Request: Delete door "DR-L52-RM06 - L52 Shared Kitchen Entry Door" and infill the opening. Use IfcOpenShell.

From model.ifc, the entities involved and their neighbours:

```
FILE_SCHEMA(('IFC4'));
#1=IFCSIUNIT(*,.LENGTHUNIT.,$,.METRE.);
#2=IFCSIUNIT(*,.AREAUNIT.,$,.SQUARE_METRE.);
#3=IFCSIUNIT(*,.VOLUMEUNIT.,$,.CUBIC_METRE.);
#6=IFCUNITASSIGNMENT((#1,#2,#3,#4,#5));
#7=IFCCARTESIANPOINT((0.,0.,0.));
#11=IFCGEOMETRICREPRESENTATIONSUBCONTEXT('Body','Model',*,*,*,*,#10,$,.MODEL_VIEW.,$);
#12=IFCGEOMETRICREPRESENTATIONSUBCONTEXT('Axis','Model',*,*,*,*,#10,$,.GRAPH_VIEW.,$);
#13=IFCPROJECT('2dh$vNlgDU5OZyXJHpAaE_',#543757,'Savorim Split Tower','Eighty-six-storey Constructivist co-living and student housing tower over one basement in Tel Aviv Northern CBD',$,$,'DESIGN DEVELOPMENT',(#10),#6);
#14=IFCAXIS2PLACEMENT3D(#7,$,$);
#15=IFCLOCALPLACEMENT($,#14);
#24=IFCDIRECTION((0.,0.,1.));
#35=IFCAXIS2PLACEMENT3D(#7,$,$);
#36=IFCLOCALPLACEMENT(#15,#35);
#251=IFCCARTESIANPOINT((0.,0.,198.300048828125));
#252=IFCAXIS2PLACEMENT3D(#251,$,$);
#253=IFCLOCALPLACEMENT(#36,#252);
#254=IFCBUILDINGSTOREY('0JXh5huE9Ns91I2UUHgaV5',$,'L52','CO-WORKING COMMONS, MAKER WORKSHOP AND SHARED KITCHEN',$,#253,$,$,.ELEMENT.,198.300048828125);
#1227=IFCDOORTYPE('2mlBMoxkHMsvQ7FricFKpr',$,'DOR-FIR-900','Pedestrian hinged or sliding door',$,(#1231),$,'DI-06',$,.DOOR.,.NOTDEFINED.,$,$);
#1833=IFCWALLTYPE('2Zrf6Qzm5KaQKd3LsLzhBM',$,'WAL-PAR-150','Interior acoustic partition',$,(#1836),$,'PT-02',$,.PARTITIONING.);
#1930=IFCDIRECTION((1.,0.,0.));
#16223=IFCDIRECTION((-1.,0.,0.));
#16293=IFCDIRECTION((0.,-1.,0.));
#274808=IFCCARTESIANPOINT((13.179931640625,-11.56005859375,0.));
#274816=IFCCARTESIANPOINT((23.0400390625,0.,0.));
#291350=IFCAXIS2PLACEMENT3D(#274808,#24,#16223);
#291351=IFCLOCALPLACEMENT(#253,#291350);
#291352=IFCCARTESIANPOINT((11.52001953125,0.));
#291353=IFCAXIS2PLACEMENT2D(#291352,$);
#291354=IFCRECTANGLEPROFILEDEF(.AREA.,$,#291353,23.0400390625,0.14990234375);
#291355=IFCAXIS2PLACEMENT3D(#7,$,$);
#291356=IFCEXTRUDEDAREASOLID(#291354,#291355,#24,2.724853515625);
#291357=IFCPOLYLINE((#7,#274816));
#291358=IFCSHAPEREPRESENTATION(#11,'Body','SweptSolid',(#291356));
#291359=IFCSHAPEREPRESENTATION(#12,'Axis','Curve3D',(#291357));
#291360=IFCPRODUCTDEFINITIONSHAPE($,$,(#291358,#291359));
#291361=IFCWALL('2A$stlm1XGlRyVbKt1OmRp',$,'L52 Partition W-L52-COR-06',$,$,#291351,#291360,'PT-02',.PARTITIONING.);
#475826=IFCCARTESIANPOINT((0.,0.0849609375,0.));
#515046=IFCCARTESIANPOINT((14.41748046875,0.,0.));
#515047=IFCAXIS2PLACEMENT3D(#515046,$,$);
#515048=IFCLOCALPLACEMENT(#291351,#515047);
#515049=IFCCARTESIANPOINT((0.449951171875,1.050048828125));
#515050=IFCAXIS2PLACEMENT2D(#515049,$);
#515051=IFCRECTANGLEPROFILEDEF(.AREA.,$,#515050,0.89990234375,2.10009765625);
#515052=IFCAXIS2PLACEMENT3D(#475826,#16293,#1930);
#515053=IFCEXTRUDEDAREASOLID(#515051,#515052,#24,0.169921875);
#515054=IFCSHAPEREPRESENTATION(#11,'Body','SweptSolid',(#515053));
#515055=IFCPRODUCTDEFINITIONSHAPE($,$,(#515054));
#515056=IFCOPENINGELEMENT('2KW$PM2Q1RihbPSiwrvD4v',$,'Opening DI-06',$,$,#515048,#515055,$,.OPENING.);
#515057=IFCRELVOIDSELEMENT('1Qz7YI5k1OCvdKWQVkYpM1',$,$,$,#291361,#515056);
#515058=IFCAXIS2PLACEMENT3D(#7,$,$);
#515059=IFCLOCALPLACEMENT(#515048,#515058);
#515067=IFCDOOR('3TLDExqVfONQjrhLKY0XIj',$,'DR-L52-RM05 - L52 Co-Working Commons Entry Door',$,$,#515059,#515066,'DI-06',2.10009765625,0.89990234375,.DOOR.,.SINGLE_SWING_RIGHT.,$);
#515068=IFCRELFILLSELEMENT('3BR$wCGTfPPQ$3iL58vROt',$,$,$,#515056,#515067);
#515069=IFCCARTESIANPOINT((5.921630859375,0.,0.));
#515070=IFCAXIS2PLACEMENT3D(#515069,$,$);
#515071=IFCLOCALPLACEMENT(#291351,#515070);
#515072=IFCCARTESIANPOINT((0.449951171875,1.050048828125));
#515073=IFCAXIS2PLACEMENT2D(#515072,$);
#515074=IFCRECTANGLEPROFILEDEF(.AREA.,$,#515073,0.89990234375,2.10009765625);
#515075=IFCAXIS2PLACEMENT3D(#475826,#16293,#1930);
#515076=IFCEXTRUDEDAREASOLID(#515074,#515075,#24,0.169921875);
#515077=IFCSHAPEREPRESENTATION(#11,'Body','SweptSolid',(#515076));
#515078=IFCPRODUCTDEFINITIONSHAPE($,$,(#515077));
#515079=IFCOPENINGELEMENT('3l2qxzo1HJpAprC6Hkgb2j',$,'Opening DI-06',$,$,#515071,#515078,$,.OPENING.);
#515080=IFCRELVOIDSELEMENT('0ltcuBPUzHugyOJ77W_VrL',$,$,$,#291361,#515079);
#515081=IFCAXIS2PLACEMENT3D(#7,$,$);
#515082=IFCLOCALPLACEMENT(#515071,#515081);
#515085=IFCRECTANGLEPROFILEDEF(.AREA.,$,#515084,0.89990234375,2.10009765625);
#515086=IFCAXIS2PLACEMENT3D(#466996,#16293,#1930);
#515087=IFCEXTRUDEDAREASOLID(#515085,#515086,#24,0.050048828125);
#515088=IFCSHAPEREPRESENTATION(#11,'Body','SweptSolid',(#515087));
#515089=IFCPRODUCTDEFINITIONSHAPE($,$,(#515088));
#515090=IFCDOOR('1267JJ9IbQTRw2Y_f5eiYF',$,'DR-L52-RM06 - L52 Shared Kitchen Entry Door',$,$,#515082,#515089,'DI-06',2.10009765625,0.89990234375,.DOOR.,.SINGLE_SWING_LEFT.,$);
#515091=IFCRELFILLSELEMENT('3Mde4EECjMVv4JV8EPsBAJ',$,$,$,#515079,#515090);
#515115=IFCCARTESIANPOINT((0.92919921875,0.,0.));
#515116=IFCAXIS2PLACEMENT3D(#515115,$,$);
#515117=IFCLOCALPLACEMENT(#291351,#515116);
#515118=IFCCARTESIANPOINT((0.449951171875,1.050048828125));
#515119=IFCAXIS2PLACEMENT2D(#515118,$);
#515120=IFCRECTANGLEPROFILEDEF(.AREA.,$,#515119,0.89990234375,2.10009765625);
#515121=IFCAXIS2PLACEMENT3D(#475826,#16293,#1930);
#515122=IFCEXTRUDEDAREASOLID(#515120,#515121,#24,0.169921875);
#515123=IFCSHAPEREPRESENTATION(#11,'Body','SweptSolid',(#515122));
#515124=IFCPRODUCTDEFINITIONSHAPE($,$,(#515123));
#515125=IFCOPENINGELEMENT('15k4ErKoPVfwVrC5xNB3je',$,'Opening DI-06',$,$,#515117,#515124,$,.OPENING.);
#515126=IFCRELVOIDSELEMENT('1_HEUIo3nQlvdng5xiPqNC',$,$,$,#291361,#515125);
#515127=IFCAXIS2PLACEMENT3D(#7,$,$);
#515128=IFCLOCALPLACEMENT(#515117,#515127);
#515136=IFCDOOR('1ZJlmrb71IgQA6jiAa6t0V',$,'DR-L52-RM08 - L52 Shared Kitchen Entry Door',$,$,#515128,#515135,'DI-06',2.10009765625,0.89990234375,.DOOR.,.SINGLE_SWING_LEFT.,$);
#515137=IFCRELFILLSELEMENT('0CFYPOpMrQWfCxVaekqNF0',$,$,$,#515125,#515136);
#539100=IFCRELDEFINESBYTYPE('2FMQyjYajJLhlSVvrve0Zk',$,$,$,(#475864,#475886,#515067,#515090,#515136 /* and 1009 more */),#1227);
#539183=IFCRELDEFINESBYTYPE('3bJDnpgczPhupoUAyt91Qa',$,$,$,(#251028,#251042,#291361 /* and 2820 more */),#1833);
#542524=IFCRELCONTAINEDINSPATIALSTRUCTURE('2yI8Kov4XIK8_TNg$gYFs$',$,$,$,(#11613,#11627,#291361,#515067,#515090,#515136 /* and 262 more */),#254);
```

```python
import ifcopenshell
import ifcopenshell.api.feature
import ifcopenshell.api.root
import ifcopenshell.geom
import ifcopenshell.util.shape

model = ifcopenshell.open("model.ifc")
settings = ifcopenshell.geom.settings()


def volume(element):
    """Net volume in cubic metres, openings subtracted."""
    shape = ifcopenshell.geom.create_shape(settings, element)
    return ifcopenshell.util.shape.get_volume(shape.geometry)


door = model.by_guid("1267JJ9IbQTRw2Y_f5eiYF")
opening = door.FillsVoids[0].RelatingOpeningElement
wall = opening.VoidsElements[0].RelatingBuildingElement
before = volume(wall)

ifcopenshell.api.root.remove_product(model, product=door)
ifcopenshell.api.feature.remove_feature(model, feature=opening)

after = volume(wall)

print(f"wall volume {before:.3f} -> {after:.3f} m3")

model.write("model_updated.ifc")
```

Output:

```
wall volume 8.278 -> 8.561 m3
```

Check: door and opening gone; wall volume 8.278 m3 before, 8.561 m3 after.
